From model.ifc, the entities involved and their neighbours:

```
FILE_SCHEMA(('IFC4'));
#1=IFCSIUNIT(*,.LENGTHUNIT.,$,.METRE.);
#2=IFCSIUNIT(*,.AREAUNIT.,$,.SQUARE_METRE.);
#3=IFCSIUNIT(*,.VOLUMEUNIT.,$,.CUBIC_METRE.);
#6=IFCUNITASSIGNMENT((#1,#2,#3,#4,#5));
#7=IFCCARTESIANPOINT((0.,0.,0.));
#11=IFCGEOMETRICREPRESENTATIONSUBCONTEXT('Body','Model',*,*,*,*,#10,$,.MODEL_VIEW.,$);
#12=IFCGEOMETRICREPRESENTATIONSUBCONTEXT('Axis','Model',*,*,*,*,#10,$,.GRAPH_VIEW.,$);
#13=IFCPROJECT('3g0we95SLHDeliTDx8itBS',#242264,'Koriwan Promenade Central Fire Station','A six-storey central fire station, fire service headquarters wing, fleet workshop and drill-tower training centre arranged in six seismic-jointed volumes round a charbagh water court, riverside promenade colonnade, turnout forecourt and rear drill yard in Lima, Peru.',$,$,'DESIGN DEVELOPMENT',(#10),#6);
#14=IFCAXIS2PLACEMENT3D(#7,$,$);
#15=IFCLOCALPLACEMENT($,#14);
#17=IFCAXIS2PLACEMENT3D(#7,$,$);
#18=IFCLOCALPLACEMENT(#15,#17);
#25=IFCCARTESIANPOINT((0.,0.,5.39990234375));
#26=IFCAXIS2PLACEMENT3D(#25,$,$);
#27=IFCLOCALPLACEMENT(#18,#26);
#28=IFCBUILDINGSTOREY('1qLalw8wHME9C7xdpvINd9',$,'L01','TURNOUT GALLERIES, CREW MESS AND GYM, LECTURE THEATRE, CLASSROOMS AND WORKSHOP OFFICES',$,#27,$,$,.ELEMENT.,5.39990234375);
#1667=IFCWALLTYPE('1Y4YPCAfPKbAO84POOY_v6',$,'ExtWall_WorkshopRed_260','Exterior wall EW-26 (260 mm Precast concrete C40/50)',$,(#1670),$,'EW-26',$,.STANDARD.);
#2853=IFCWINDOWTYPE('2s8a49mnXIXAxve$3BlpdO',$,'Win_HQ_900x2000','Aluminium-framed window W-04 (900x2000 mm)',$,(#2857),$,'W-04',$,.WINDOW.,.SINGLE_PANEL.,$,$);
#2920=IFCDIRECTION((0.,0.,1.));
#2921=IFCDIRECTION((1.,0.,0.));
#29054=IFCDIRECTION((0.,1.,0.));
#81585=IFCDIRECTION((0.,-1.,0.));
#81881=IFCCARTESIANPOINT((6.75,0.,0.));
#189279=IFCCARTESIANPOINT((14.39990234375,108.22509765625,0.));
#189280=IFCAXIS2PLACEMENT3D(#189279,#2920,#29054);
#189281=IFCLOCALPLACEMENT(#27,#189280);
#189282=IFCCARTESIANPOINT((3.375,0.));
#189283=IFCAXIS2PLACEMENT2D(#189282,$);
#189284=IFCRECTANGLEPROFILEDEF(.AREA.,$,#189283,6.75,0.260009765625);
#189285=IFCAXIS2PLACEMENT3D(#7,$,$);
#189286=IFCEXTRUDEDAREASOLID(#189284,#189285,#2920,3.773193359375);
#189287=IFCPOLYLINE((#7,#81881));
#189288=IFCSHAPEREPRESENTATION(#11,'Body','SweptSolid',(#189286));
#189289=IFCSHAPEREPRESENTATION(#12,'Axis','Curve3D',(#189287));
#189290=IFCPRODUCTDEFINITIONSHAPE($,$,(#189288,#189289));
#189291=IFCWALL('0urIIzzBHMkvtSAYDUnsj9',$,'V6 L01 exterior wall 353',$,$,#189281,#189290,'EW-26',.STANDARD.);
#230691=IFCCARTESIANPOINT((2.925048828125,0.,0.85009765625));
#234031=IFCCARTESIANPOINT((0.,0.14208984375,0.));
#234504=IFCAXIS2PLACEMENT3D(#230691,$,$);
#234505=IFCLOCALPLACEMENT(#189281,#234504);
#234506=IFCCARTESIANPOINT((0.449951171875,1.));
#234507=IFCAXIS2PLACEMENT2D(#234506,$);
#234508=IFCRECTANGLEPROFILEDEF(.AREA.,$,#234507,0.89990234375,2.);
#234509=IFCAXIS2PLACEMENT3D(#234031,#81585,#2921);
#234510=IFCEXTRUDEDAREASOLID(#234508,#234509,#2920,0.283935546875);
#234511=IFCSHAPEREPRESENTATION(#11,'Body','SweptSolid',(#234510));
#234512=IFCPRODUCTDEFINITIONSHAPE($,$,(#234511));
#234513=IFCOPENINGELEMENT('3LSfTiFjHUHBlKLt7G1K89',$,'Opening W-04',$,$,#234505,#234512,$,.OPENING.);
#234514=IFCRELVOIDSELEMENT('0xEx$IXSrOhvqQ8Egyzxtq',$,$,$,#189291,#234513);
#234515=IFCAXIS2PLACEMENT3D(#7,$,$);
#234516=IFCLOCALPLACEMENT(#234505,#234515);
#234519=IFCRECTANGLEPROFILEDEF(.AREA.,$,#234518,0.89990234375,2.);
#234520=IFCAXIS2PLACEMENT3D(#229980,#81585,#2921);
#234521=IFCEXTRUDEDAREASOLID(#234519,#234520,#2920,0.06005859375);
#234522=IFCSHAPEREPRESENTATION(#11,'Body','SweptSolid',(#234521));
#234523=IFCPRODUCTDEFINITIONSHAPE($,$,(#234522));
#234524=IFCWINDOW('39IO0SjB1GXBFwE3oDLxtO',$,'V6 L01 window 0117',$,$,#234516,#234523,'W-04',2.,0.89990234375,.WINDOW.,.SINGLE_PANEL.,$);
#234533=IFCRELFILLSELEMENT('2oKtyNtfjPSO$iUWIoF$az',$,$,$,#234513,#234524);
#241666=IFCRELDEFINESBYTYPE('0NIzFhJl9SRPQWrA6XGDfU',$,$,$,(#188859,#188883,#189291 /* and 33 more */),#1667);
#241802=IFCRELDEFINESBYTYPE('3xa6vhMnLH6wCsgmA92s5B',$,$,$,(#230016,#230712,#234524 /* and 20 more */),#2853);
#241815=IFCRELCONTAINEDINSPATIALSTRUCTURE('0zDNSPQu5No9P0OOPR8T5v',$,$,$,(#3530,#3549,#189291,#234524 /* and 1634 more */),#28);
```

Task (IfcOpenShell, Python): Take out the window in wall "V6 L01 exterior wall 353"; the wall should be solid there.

```python
import ifcopenshell
import ifcopenshell.api.feature
import ifcopenshell.api.root
import ifcopenshell.geom
import ifcopenshell.util.shape

model = ifcopenshell.open("model.ifc")
settings = ifcopenshell.geom.settings()


def volume(element):
    """Net volume in cubic metres, openings subtracted."""
    shape = ifcopenshell.geom.create_shape(settings, element)
    return ifcopenshell.util.shape.get_volume(shape.geometry)


window = model.by_guid("39IO0SjB1GXBFwE3oDLxtO")
opening = window.FillsVoids[0].RelatingOpeningElement
wall = opening.VoidsElements[0].RelatingBuildingElement
before = volume(wall)

ifcopenshell.api.root.remove_product(model, product=window)
ifcopenshell.api.feature.remove_feature(model, feature=opening)

after = volume(wall)

print(f"wall volume {before:.3f} -> {after:.3f} m3")

model.write("model_updated.ifc")
```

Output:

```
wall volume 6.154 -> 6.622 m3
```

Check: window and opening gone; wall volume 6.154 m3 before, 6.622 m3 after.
